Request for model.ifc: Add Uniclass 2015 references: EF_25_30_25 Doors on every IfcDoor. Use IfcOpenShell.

First a look at what the model holds.

```python
import ifcopenshell

model = ifcopenshell.open("model.ifc")
print(model.schema)
print("classifications:", [c.Name for c in model.by_type("IfcClassification")])
for ifc_class in ("IfcDoor", "IfcRoof", "IfcStair", "IfcWall", "IfcWindow"):
    print(ifc_class, len(model.by_type(ifc_class)))
```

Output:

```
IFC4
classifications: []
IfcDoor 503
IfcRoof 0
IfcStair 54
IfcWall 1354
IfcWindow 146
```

```python
import ifcopenshell
import ifcopenshell.api.classification

model = ifcopenshell.open("model.ifc")

system = ifcopenshell.api.classification.add_classification(model, classification="Uniclass 2015")

codes = {
    "IfcDoor": ("EF_25_30_25", "Doors"),
}
for ifc_class, (code, name) in codes.items():
    products = model.by_type(ifc_class)
    ifcopenshell.api.classification.add_reference(
        model, products=products, classification=system, identification=code, name=name
    )
    print(code, len(products))

model.write("model_updated.ifc")
```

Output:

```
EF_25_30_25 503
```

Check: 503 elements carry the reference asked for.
